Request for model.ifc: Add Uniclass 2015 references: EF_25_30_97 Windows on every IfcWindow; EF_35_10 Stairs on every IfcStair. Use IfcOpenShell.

First a look at what the model holds.

```python
import ifcopenshell

model = ifcopenshell.open("model.ifc")
print(model.schema)
print("classifications:", [c.Name for c in model.by_type("IfcClassification")])
for ifc_class in ("IfcDoor", "IfcRoof", "IfcStair", "IfcWall", "IfcWindow"):
    print(ifc_class, len(model.by_type(ifc_class)))
```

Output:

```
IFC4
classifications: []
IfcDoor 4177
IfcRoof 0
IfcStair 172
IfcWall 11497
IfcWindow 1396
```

```python
import ifcopenshell
import ifcopenshell.api.classification

model = ifcopenshell.open("model.ifc")

system = ifcopenshell.api.classification.add_classification(model, classification="Uniclass 2015")

codes = {
    "IfcWindow": ("EF_25_30_97", "Windows"),
    "IfcStair": ("EF_35_10", "Stairs"),
}
for ifc_class, (code, name) in codes.items():
    products = model.by_type(ifc_class)
    ifcopenshell.api.classification.add_reference(
        model, products=products, classification=system, identification=code, name=name
    )
    print(code, len(products))

model.write("model_v2.ifc")
```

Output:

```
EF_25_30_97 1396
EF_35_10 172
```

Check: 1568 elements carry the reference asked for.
